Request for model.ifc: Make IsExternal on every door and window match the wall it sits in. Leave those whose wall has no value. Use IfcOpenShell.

First a look at what the model holds.

```python
import ifcopenshell
import ifcopenshell.util.element

model = ifcopenshell.open("model.ifc")
print(model.schema)
seen = {}
for e in model.by_type("IfcDoor") + model.by_type("IfcWindow"):
    if not e.FillsVoids:
        continue
    host = e.FillsVoids[0].RelatingOpeningElement.VoidsElements[0].RelatingBuildingElement
    own = ifcopenshell.util.element.get_pset(e, f"Pset_{e.is_a()[3:].removesuffix('StandardCase')}Common", "IsExternal")
    wall = ifcopenshell.util.element.get_pset(host, "Pset_WallCommon", "IsExternal")
    seen[e.is_a(), own, wall] = seen.get((e.is_a(), own, wall), 0) + 1
for (cls, own, wall), count in sorted(seen.items(), key=str):
    print(count, cls, "IsExternal:", own, "| host wall:", wall)
```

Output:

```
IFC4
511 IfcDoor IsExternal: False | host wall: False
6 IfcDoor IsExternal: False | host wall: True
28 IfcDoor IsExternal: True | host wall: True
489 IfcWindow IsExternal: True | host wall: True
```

```python
import ifcopenshell
import ifcopenshell.api.pset
import ifcopenshell.util.element

model = ifcopenshell.open("model.ifc")

count = 0
for ifc_class, pset_name in (("IfcDoor", "Pset_DoorCommon"), ("IfcWindow", "Pset_WindowCommon")):
    for e in model.by_type(ifc_class):
        if not e.FillsVoids:
            continue
        host = e.FillsVoids[0].RelatingOpeningElement.VoidsElements[0].RelatingBuildingElement
        external = ifcopenshell.util.element.get_pset(host, "Pset_WallCommon", "IsExternal")
        if external is None or ifcopenshell.util.element.get_pset(e, pset_name, "IsExternal") == external:
            continue
        pset = ifcopenshell.api.pset.add_pset(model, product=e, name=pset_name)
        ifcopenshell.api.pset.edit_pset(model, pset=pset, properties={"IsExternal": external})
        count += 1

print(count, "updated")

model.write("model_rev.ifc")
```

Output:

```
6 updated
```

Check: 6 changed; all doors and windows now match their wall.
